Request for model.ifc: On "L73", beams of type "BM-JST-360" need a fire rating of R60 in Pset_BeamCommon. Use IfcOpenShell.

First a look at what the model holds.

```python
import ifcopenshell
import ifcopenshell.util.element

model = ifcopenshell.open("model.ifc")
print(model.schema)
storey = next(s for s in model.by_type("IfcBuildingStorey") if s.Name == "L73")
beams = [e for e in ifcopenshell.util.element.get_decomposition(storey) if e.is_a("IfcBeam")]
seen = {}
for e in beams:
    element_type = ifcopenshell.util.element.get_type(e)
    key = (element_type.Name if element_type != e and element_type else None, ifcopenshell.util.element.get_pset(e, "Pset_BeamCommon", "FireRating"))
    seen[key] = seen.get(key, 0) + 1
for (name, value), count in sorted(seen.items(), key=str):
    print(count, "x", name, "|", value)
```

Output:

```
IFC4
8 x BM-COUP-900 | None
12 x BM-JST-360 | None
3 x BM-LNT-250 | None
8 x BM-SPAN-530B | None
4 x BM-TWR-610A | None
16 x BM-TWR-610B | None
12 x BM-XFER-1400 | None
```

```python
import ifcopenshell
import ifcopenshell.api.pset
import ifcopenshell.util.element

model = ifcopenshell.open("model.ifc")

storey = next(s for s in model.by_type("IfcBuildingStorey") if s.Name == "L73")
beams = [e for e in ifcopenshell.util.element.get_decomposition(storey) if e.is_a("IfcBeam")]

count = 0
for e in beams:
    element_type = ifcopenshell.util.element.get_type(e)
    if element_type in (None, e) or element_type.Name != "BM-JST-360":
        continue
    found = ifcopenshell.util.element.get_pset(e, "Pset_BeamCommon", should_inherit=False)
    if found:
        pset = model.by_id(found["id"])
        if len(ifcopenshell.util.element.get_elements_by_pset(pset)) > 1:
            pset = ifcopenshell.api.pset.unshare_pset(model, products=[e], pset=pset)[0]
    else:
        pset = ifcopenshell.api.pset.add_pset(model, product=e, name="Pset_BeamCommon")
    ifcopenshell.api.pset.edit_pset(model, pset=pset, properties={"FireRating": "R60"})
    count += 1

print(count, "beams updated")

model.write("model-out.ifc")
```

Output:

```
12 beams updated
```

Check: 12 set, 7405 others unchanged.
